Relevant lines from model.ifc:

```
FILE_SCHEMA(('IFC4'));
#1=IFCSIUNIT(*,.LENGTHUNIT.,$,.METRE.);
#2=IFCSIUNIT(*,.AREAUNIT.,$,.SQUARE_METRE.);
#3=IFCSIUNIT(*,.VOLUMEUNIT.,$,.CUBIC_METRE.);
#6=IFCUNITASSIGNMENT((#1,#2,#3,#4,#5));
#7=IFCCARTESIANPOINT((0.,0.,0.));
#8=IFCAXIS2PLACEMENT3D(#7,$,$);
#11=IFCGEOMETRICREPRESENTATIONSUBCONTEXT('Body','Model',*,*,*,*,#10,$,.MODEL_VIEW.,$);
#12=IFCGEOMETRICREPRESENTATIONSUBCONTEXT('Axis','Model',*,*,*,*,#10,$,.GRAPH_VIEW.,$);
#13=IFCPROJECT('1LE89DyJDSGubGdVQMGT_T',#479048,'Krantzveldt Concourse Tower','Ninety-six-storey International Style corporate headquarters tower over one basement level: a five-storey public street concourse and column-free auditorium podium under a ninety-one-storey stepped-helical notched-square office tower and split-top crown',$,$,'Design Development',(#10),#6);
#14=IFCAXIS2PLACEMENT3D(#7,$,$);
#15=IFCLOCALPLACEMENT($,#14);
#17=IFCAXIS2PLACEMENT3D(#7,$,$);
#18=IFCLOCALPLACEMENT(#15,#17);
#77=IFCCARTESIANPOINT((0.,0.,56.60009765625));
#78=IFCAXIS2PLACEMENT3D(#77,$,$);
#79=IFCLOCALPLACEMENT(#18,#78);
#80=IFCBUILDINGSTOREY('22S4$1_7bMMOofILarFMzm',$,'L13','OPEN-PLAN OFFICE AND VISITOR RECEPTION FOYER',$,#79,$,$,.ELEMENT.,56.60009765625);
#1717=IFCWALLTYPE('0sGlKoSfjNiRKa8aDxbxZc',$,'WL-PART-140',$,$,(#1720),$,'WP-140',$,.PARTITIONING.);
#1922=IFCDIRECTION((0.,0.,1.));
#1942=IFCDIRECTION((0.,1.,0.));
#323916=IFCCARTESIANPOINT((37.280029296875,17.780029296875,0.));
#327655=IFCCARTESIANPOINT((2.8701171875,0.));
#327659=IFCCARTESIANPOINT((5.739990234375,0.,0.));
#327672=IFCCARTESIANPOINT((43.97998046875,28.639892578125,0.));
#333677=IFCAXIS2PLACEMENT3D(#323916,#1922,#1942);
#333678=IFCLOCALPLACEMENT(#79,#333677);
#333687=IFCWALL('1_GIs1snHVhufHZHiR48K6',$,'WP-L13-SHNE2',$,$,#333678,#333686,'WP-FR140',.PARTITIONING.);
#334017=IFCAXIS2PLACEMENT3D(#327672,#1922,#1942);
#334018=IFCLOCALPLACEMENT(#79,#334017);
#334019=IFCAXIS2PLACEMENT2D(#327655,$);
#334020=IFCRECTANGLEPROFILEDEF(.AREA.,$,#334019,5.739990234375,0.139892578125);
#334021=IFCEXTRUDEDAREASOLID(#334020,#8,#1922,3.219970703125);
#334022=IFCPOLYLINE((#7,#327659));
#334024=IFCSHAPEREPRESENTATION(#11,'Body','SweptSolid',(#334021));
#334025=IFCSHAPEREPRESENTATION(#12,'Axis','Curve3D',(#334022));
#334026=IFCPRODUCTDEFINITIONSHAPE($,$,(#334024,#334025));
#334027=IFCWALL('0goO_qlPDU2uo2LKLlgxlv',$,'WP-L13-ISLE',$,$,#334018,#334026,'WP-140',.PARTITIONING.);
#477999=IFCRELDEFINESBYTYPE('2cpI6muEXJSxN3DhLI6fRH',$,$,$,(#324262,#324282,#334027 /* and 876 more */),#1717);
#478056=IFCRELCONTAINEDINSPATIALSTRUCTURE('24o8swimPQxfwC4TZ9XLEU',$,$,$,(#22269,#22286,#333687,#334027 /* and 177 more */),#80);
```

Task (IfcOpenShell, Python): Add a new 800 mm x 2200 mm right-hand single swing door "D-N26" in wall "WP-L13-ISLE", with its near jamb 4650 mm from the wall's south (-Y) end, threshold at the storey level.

```python
import numpy as np
import ifcopenshell
import ifcopenshell.api.feature
import ifcopenshell.api.geometry
import ifcopenshell.api.root
import ifcopenshell.api.spatial
import ifcopenshell.geom
import ifcopenshell.util.element
import ifcopenshell.util.placement
import ifcopenshell.util.representation
import ifcopenshell.util.shape
import ifcopenshell.util.unit

model = ifcopenshell.open("model.ifc")
unit_scale = ifcopenshell.util.unit.calculate_unit_scale(model)
settings = ifcopenshell.geom.settings()


def volume(element):
    """Net volume in cubic metres, openings subtracted."""
    shape = ifcopenshell.geom.create_shape(settings, element)
    return ifcopenshell.util.shape.get_volume(shape.geometry)


wall = model.by_guid("0goO_qlPDU2uo2LKLlgxlv")
storey = ifcopenshell.util.element.get_container(wall, ifc_class="IfcBuildingStorey")
context = ifcopenshell.util.representation.get_context(model, "Model", "Body", "MODEL_VIEW")
before = volume(wall)

width, height, from_end, sill = 0.8, 2.2, 4.65, 0.0  # metres

# The wall runs along its own X axis, and the end named is its -X end.
wall_shape = ifcopenshell.geom.create_shape(settings, wall)
x, y, z = ifcopenshell.util.shape.get_vertices(wall_shape.geometry).T
start = x.min() + from_end
face, thickness = float(y.min()), float(y.max() - y.min())
wall_matrix = ifcopenshell.util.placement.get_local_placement(wall.ObjectPlacement)
level = ifcopenshell.util.placement.get_local_placement(storey.ObjectPlacement)[2, 3]


def in_wall(x, y):
    """Placement at x, y metres in the wall's axes, at sill height."""
    matrix = wall_matrix.copy()
    matrix[:, 3] = wall_matrix @ np.array([x / unit_scale, y / unit_scale, 0.0, 1.0])
    matrix[2, 3] = level + sill / unit_scale
    return matrix


# Opening: a box that overshoots both wall faces by 50 mm.
opening = ifcopenshell.api.root.create_entity(model, ifc_class="IfcOpeningElement", predefined_type="OPENING")
box = ifcopenshell.api.geometry.add_wall_representation(
    model, context=context, length=width, height=height, thickness=thickness + 0.1
)
ifcopenshell.api.geometry.assign_representation(model, product=opening, representation=box)
ifcopenshell.api.geometry.edit_object_placement(model, product=opening, matrix=in_wall(start, face - 0.05), is_si=False)
ifcopenshell.api.feature.add_feature(model, feature=opening, element=wall)

door = ifcopenshell.api.root.create_entity(model, ifc_class="IfcDoor", name="D-N26", predefined_type="DOOR")
door.OverallWidth, door.OverallHeight = width / unit_scale, height / unit_scale
door.OperationType = "SINGLE_SWING_RIGHT"
body = ifcopenshell.api.geometry.add_door_representation(
    model,
    context=context,
    overall_width=door.OverallWidth,
    overall_height=door.OverallHeight,
    operation_type="SINGLE_SWING_RIGHT",
    lining_properties={"LiningDepth": thickness / unit_scale, "ThresholdDepth": thickness / unit_scale},
)
ifcopenshell.api.geometry.assign_representation(model, product=door, representation=body)
ifcopenshell.api.spatial.assign_container(model, products=[door], relating_structure=storey)
ifcopenshell.api.feature.add_filling(model, opening=opening, element=door)

# The lining spans the wall, so the door starts at the wall face.
ifcopenshell.api.geometry.edit_object_placement(model, product=door, matrix=in_wall(start, face), is_si=False)

after = volume(wall)

print(f"wall volume {before:.3f} -> {after:.3f} m3")

model.write("model-out.ifc")
```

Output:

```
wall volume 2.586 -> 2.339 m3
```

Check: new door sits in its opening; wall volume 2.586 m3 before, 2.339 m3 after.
